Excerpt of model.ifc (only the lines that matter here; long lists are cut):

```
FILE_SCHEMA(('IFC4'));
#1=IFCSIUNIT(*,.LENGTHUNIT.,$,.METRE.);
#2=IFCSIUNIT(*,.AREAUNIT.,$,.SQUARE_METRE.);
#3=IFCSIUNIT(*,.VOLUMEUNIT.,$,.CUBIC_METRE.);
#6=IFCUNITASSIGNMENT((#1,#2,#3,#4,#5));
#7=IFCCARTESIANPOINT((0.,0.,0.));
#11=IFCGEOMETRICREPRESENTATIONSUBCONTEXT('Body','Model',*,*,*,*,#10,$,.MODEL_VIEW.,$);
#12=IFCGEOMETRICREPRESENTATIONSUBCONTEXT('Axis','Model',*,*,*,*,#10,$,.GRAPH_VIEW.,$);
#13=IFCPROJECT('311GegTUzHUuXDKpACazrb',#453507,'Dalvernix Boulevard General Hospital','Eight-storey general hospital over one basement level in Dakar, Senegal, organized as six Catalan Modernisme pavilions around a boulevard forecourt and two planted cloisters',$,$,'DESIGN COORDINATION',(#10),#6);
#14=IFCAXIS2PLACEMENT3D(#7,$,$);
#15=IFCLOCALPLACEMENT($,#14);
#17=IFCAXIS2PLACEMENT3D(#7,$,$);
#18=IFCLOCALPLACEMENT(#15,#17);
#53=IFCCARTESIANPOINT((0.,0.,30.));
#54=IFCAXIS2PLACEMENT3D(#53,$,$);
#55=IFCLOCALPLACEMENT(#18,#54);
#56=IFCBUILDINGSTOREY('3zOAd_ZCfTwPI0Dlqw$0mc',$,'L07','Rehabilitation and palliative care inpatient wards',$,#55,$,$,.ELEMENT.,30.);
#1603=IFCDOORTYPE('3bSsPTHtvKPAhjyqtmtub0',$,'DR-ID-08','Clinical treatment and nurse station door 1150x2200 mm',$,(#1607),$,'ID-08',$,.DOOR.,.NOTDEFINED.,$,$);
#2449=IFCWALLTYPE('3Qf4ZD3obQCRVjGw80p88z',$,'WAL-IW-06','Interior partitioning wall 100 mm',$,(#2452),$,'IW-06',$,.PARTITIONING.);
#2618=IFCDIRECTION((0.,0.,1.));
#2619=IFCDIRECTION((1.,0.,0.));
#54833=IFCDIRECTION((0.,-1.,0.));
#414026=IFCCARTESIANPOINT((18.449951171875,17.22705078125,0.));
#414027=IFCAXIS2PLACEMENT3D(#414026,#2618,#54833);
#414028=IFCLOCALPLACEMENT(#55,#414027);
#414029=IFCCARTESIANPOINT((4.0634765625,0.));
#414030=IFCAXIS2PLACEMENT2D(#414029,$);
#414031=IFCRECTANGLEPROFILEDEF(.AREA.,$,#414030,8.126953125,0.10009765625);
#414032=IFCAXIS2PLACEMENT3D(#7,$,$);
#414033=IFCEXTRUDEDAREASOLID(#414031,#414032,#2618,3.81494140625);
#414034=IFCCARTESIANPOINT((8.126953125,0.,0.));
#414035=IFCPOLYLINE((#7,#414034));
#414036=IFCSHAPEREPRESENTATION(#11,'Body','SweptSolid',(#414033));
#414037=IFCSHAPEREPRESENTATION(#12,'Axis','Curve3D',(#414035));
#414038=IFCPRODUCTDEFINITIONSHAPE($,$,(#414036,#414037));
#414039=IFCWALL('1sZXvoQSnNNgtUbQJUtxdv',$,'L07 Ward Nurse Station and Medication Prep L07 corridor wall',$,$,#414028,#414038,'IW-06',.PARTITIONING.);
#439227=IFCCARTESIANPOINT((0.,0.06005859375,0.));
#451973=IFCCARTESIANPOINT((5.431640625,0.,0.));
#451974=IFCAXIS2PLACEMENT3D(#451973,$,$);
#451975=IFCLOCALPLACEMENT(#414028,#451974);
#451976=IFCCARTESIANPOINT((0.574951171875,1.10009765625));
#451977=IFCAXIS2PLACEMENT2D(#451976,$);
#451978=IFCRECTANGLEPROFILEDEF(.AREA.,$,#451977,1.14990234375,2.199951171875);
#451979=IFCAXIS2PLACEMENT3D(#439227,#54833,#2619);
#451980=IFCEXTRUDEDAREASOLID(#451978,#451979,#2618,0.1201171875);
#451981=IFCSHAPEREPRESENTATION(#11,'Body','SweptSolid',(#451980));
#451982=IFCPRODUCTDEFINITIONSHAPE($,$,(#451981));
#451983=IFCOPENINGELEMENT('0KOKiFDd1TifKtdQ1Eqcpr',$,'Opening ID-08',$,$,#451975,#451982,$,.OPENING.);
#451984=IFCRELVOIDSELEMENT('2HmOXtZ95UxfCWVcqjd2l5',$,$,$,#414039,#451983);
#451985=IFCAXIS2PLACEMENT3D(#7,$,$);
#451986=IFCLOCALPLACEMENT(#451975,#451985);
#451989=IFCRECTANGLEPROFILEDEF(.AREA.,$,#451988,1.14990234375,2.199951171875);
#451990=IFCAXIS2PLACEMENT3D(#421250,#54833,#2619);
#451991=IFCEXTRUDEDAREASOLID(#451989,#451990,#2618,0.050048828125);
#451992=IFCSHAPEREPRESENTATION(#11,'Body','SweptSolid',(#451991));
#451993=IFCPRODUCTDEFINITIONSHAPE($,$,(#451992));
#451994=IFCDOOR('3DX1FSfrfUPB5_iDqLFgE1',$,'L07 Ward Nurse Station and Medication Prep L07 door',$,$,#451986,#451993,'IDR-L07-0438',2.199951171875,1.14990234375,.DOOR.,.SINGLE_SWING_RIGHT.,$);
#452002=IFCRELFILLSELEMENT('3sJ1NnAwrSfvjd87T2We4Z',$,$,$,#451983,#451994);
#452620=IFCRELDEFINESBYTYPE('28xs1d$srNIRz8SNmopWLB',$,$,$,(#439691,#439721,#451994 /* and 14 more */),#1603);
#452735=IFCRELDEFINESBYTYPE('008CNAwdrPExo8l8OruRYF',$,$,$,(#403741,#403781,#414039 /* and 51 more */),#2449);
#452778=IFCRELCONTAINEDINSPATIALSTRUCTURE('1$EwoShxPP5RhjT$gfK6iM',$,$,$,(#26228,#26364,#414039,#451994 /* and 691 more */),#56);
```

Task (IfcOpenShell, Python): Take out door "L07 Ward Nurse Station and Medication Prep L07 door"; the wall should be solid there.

```python
import ifcopenshell
import ifcopenshell.api.feature
import ifcopenshell.api.root
import ifcopenshell.geom
import ifcopenshell.util.shape

model = ifcopenshell.open("model.ifc")
settings = ifcopenshell.geom.settings()


def volume(element):
    """Net volume in cubic metres, openings subtracted."""
    shape = ifcopenshell.geom.create_shape(settings, element)
    return ifcopenshell.util.shape.get_volume(shape.geometry)


door = model.by_guid("3DX1FSfrfUPB5_iDqLFgE1")
opening = door.FillsVoids[0].RelatingOpeningElement
wall = opening.VoidsElements[0].RelatingBuildingElement
before = volume(wall)

ifcopenshell.api.root.remove_product(model, product=door)
ifcopenshell.api.feature.remove_feature(model, feature=opening)

after = volume(wall)

print(f"wall volume {before:.3f} -> {after:.3f} m3")

model.write("model-out.ifc")
```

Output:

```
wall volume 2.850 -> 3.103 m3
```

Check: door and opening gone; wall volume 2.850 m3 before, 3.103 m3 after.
